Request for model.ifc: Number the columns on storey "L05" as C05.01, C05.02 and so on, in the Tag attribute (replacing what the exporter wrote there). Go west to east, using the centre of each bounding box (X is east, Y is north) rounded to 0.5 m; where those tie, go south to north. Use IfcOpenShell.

First a look at what the model holds.

```python
import ifcopenshell
import ifcopenshell.util.element
import ifcopenshell.util.placement

model = ifcopenshell.open("model.ifc")
print(model.schema)
storey = next(s for s in model.by_type("IfcBuildingStorey") if s.Name == "L05")
columns = [e for e in ifcopenshell.util.element.get_decomposition(storey) if e.is_a("IfcColumn")]
for e in sorted(columns, key=lambda e: e.id()):
    origin = ifcopenshell.util.placement.get_local_placement(e.ObjectPlacement)[:3, 3]
    print(e.id(), e.Tag, e.Name, origin.round(2) + 0.0, sep=" | ")
```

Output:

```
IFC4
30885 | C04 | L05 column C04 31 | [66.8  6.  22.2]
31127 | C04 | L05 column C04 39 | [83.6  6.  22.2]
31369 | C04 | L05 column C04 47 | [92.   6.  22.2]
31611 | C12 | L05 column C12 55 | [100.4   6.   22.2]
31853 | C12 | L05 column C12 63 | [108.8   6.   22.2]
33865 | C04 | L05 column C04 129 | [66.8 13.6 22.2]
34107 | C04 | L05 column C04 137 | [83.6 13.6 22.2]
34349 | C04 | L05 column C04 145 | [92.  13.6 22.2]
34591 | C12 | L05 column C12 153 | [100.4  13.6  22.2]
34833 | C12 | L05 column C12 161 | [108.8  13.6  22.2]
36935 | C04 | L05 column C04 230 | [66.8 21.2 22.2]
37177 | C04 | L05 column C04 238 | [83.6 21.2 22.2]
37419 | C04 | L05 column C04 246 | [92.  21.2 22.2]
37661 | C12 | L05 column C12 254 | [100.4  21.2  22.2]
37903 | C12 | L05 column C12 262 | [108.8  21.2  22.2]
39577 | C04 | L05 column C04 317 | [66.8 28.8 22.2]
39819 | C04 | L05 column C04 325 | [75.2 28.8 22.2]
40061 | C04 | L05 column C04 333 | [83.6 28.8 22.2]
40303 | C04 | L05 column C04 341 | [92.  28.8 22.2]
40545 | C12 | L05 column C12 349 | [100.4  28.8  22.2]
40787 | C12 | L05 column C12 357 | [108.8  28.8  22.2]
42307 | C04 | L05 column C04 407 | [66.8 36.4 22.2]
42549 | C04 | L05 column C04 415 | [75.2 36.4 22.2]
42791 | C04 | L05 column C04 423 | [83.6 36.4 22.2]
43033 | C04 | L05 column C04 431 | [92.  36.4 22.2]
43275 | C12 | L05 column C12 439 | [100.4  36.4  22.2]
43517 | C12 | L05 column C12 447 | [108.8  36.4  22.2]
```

```python
import ifcopenshell
import ifcopenshell.geom
import ifcopenshell.util.element
import ifcopenshell.util.shape

model = ifcopenshell.open("model.ifc")
settings = ifcopenshell.geom.settings()
settings.set("use-world-coords", True)


def centre(element):
    shape = ifcopenshell.geom.create_shape(settings, element)
    return ifcopenshell.util.shape.get_bbox_centroid(shape.geometry)


storey = next(s for s in model.by_type("IfcBuildingStorey") if s.Name == "L05")
columns = [e for e in ifcopenshell.util.element.get_decomposition(storey) if e.is_a("IfcColumn")]

# Insertion points can sit at a corner or the storey origin, so sort by the geometry (in metres).
centres = {e: centre(e) for e in columns}
columns.sort(key=lambda e: (round(centres[e][0] / 0.5), centres[e][1]))

for i, e in enumerate(columns, start=1):
    number = f"C05.{i:02d}"
    e.Tag = number
    print(e.id(), number)

model.write("model_rev.ifc")
```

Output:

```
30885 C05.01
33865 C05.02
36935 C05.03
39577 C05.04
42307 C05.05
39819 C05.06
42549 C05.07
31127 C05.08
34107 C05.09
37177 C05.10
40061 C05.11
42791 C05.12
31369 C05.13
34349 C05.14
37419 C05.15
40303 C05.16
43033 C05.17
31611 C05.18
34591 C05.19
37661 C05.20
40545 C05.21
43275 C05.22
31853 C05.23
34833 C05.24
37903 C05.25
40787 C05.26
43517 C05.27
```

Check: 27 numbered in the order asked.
